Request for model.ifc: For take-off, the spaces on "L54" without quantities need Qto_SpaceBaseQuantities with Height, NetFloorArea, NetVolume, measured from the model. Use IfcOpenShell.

First a look at what the model holds.

```python
import ifcopenshell
import ifcopenshell.util.element
import ifcopenshell.util.unit

model = ifcopenshell.open("model.ifc")
print(model.schema)
for unit_type in ("LENGTHUNIT", "AREAUNIT", "VOLUMEUNIT"):
    print(unit_type, ifcopenshell.util.unit.calculate_unit_scale(model, unit_type))
storey = next(s for s in model.by_type("IfcBuildingStorey") if s.Name == "L54")
spaces = [e for e in ifcopenshell.util.element.get_decomposition(storey) if e.is_a("IfcSpace")]
for e in sorted(spaces, key=lambda e: e.id()):
    print(e.id(), e.is_a(), e.Name, list(ifcopenshell.util.element.get_psets(e, qtos_only=True)), sep=" | ")
```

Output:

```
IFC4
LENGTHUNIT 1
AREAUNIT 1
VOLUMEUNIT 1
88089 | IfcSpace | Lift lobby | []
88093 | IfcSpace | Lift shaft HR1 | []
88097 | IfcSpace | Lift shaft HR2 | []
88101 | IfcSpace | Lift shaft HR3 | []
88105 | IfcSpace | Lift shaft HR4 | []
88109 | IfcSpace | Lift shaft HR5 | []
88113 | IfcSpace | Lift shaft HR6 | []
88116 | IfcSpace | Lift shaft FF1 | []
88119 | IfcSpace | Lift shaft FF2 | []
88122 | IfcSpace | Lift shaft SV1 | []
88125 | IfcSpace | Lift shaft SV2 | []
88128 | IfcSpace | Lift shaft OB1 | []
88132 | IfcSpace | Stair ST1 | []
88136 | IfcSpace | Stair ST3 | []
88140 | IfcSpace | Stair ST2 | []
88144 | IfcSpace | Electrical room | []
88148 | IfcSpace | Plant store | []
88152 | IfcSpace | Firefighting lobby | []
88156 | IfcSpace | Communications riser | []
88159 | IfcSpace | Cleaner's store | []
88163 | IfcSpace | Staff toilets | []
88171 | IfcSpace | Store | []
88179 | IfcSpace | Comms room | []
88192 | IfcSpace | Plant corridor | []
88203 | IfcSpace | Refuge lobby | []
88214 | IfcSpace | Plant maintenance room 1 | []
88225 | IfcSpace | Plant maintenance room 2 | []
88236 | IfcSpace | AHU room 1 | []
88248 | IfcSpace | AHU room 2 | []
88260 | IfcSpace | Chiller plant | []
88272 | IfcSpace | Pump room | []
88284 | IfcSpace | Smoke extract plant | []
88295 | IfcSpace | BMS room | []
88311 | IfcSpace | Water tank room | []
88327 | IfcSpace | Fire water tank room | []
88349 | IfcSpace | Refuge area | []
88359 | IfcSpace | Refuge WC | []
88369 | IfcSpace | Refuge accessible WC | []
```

```python
import ifcopenshell
import ifcopenshell.api.pset
import ifcopenshell.geom
import ifcopenshell.util.element
import ifcopenshell.util.shape
import ifcopenshell.util.unit

model = ifcopenshell.open("model.ifc")
unit_scale = ifcopenshell.util.unit.calculate_unit_scale(model)
area_scale = ifcopenshell.util.unit.calculate_unit_scale(model, "AREAUNIT")
volume_scale = ifcopenshell.util.unit.calculate_unit_scale(model, "VOLUMEUNIT")
settings = ifcopenshell.geom.settings()

storey = next(s for s in model.by_type("IfcBuildingStorey") if s.Name == "L54")
spaces = [e for e in ifcopenshell.util.element.get_decomposition(storey) if e.is_a("IfcSpace")]

for e in sorted(spaces, key=lambda e: e.id()):
    if ifcopenshell.util.element.get_psets(e, qtos_only=True, should_inherit=False):
        continue
    # Geometry comes back in metres, in the element's own axes.
    shape = ifcopenshell.geom.create_shape(settings, e)
    values = {
        "Height": ifcopenshell.util.shape.get_z(shape.geometry) / unit_scale,
        "NetFloorArea": ifcopenshell.util.shape.get_footprint_area(shape.geometry) / area_scale,
        "NetVolume": ifcopenshell.util.shape.get_volume(shape.geometry) / volume_scale,
    }
    qto = ifcopenshell.api.pset.add_qto(model, product=e, name="Qto_SpaceBaseQuantities")
    ifcopenshell.api.pset.edit_qto(model, qto=qto, properties=values)
    print(e.id(), {k: round(v, 3) for k, v in values.items()})

model.write("model_updated.ifc")
```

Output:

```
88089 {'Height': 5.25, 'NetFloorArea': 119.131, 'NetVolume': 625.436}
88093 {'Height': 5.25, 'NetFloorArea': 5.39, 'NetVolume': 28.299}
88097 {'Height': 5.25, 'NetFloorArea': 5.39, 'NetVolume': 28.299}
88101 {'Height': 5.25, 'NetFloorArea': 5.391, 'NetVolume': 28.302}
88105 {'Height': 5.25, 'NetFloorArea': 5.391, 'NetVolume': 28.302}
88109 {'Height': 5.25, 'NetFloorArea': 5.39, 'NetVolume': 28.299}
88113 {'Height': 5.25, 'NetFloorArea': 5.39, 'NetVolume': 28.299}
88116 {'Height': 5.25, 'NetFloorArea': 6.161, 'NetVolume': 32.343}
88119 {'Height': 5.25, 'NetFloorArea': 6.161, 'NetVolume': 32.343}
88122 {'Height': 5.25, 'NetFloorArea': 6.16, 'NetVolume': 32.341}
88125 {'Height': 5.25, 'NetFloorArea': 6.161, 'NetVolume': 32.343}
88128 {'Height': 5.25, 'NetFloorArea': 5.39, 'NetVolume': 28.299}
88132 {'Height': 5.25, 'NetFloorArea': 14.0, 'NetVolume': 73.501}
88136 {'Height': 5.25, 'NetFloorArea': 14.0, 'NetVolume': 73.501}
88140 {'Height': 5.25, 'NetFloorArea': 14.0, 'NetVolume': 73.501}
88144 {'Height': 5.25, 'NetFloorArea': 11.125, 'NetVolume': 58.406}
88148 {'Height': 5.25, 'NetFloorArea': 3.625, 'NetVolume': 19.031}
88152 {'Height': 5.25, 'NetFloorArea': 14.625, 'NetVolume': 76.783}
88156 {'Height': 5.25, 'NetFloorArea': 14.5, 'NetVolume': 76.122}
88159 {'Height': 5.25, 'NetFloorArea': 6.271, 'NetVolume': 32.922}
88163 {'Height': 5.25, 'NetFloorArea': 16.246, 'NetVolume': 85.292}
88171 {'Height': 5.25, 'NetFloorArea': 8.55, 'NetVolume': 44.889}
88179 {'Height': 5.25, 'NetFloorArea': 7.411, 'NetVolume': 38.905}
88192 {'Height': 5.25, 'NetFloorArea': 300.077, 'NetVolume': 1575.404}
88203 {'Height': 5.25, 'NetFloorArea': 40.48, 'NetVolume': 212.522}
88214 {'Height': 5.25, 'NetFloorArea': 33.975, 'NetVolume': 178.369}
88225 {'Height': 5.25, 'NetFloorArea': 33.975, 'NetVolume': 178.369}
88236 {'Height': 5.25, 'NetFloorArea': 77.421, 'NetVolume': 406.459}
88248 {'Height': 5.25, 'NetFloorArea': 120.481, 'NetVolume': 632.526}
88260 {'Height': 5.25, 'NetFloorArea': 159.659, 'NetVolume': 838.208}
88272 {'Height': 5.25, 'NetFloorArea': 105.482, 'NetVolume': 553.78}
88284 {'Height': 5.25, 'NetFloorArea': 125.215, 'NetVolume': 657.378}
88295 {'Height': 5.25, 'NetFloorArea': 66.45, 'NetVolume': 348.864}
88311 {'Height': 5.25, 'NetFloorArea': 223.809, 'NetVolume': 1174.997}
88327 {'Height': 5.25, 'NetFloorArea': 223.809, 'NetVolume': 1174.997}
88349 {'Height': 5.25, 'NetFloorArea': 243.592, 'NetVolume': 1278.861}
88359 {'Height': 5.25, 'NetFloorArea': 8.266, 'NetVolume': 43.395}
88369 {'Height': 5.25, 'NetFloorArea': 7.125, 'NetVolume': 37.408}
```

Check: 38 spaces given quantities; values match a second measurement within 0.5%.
